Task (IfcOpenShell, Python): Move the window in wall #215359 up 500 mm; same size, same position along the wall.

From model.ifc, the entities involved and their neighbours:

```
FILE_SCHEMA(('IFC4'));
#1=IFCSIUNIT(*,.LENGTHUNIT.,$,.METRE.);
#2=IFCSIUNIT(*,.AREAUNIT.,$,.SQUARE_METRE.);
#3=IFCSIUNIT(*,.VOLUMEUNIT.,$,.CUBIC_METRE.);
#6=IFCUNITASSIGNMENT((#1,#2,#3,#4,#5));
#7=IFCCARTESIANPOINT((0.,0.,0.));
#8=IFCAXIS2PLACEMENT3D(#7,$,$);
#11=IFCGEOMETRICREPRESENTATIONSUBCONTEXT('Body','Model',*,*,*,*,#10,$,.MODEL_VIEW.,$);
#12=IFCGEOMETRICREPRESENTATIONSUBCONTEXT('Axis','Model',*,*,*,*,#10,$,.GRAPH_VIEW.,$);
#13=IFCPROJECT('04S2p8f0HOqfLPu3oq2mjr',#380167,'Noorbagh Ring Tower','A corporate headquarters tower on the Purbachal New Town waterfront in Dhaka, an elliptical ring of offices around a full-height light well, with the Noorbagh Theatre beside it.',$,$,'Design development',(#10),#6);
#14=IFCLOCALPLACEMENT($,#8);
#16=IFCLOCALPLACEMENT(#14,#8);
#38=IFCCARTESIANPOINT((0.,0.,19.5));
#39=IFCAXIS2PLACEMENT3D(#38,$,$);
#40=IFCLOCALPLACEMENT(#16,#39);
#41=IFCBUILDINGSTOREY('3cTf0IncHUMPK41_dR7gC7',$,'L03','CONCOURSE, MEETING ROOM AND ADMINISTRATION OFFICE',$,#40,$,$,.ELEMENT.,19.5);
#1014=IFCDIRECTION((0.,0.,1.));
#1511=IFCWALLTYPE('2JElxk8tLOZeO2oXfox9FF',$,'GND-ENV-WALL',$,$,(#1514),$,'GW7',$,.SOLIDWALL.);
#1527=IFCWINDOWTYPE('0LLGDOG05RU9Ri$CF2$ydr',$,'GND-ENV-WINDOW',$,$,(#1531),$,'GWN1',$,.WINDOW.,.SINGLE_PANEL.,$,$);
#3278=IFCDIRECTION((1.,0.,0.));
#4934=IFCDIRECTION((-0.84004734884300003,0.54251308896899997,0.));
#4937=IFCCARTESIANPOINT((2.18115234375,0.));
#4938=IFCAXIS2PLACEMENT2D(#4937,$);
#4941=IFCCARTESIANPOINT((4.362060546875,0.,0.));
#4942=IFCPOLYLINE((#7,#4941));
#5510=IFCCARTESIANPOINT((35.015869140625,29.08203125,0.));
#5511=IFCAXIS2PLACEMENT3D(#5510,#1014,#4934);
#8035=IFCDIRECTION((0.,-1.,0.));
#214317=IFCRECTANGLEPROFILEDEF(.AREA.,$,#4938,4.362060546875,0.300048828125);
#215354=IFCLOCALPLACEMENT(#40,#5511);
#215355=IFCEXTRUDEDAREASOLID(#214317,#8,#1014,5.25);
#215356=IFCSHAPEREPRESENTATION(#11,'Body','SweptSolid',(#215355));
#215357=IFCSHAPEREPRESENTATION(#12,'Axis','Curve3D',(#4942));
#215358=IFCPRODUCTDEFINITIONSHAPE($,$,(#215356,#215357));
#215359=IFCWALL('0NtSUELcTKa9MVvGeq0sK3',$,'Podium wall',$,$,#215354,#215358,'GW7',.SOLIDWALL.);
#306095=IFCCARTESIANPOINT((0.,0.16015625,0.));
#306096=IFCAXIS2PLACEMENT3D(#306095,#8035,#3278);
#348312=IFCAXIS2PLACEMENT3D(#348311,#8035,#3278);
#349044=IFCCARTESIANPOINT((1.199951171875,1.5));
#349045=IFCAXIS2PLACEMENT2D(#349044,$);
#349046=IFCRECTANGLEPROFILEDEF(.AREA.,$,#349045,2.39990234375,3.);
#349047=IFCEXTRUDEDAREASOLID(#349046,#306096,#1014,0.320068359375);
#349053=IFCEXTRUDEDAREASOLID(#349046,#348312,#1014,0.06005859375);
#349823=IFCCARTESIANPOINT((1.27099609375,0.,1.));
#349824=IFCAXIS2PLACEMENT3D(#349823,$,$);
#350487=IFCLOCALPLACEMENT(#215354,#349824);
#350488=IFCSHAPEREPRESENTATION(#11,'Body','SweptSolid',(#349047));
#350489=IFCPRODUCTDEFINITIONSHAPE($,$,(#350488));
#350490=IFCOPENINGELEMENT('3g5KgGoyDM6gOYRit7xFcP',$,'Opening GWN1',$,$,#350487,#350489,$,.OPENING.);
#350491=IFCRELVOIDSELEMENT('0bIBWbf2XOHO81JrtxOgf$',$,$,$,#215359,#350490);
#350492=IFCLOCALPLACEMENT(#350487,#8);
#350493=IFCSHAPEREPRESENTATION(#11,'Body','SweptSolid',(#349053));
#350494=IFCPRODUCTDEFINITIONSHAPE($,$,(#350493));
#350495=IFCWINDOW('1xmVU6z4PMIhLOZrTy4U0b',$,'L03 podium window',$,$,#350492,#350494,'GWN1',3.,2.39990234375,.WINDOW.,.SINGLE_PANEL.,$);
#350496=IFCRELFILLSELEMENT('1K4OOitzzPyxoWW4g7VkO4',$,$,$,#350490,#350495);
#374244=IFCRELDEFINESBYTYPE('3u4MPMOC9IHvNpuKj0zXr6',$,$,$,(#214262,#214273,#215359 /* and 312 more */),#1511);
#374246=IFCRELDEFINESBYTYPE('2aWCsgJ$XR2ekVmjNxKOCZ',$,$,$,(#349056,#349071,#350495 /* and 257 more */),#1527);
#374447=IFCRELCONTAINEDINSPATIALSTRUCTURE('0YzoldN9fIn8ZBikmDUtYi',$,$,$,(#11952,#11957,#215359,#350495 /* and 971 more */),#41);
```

```python
import numpy as np
import ifcopenshell
import ifcopenshell.api.geometry
import ifcopenshell.util.placement
import ifcopenshell.util.unit

model = ifcopenshell.open("model.ifc")
unit_scale = ifcopenshell.util.unit.calculate_unit_scale(model)

window = model.by_guid("1xmVU6z4PMIhLOZrTy4U0b")
opening = window.FillsVoids[0].RelatingOpeningElement
dz = 0.5

shift = np.array([0.0, 0.0, dz])
# The window is placed relative to its opening, so it follows when the opening moves.
matrix = ifcopenshell.util.placement.get_local_placement(opening.ObjectPlacement)
matrix[:3, 3] += shift
ifcopenshell.api.geometry.edit_object_placement(
    model, product=opening, matrix=matrix, is_si=False, should_transform_children=True
)

print(f"moved by {dz * unit_scale:+.3f} m")

model.write("model_updated.ifc")
```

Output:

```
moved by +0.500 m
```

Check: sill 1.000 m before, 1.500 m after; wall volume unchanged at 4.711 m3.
